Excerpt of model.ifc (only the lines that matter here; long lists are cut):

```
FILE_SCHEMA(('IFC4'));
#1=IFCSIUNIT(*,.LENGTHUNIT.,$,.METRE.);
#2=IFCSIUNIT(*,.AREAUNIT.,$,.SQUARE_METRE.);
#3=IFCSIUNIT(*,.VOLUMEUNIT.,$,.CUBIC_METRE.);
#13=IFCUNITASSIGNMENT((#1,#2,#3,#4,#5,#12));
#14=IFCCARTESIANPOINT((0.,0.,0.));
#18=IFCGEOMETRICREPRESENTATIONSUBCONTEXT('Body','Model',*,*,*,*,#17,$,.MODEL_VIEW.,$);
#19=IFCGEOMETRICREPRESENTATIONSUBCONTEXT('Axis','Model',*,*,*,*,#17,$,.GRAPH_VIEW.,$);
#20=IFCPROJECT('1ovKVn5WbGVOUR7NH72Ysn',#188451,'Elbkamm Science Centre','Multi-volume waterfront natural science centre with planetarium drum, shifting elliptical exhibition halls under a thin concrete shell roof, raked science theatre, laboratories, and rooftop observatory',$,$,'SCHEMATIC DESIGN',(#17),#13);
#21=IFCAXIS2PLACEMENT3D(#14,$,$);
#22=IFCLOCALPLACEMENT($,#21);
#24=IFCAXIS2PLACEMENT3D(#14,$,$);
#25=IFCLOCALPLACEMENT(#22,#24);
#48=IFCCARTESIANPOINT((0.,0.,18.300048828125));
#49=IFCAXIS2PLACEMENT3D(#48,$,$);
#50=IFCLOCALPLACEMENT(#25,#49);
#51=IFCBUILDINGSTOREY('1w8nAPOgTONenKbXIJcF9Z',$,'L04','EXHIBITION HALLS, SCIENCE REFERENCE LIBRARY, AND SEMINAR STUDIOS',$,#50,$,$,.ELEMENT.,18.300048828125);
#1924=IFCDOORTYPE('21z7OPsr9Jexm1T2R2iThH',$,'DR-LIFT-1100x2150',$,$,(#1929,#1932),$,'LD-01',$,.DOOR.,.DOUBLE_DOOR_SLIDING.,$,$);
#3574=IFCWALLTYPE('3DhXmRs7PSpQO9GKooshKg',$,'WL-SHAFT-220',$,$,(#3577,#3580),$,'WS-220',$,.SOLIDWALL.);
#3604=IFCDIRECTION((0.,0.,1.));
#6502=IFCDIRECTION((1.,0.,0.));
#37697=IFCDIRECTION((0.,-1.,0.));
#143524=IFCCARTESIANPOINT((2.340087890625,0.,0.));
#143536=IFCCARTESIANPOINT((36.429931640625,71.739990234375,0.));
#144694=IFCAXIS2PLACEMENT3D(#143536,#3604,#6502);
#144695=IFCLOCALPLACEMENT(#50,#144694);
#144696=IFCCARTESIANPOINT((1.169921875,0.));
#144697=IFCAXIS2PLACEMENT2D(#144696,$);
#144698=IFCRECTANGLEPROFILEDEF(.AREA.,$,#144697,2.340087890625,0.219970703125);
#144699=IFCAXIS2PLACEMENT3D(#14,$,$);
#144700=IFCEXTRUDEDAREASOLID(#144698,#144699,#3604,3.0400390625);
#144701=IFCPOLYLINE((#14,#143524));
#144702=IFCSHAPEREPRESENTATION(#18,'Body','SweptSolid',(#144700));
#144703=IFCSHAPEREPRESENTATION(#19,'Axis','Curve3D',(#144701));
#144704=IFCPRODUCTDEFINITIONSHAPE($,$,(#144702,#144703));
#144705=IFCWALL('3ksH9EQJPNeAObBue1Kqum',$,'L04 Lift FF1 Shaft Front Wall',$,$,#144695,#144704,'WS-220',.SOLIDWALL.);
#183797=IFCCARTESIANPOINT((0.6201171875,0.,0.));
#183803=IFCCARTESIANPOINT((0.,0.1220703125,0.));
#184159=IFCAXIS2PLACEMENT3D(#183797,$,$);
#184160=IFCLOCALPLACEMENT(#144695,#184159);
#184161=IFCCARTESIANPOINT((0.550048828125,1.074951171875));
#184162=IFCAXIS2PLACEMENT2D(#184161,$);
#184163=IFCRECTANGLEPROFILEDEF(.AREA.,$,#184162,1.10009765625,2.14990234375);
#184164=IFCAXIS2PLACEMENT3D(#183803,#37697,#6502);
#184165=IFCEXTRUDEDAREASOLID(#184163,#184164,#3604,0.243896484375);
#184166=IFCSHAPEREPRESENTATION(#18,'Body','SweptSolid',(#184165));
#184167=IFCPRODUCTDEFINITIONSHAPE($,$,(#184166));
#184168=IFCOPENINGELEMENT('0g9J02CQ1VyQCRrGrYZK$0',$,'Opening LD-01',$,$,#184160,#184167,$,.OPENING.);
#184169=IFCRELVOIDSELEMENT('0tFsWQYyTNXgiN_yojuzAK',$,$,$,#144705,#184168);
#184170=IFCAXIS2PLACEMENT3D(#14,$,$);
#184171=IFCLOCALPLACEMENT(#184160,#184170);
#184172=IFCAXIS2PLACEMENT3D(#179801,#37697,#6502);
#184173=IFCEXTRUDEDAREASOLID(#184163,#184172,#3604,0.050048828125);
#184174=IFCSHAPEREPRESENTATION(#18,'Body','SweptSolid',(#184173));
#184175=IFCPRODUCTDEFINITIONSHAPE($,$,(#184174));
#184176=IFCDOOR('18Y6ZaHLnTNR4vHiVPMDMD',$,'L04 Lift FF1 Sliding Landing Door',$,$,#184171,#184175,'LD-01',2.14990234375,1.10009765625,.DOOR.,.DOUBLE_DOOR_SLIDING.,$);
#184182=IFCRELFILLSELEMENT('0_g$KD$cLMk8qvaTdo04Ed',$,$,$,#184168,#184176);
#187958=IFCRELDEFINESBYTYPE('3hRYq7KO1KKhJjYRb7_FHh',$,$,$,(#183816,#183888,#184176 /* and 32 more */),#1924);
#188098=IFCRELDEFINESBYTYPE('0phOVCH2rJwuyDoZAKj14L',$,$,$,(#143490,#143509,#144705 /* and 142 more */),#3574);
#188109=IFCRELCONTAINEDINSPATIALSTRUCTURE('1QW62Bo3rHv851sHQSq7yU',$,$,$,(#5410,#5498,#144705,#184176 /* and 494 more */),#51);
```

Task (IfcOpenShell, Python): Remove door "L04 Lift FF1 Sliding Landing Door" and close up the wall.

```python
import ifcopenshell
import ifcopenshell.api.feature
import ifcopenshell.api.root
import ifcopenshell.geom
import ifcopenshell.util.shape

model = ifcopenshell.open("model.ifc")
settings = ifcopenshell.geom.settings()


def volume(element):
    """Net volume in cubic metres, openings subtracted."""
    shape = ifcopenshell.geom.create_shape(settings, element)
    return ifcopenshell.util.shape.get_volume(shape.geometry)


door = model.by_id(184176)
opening = door.FillsVoids[0].RelatingOpeningElement
wall = opening.VoidsElements[0].RelatingBuildingElement
before = volume(wall)

ifcopenshell.api.root.remove_product(model, product=door)
ifcopenshell.api.feature.remove_feature(model, feature=opening)

after = volume(wall)

print(f"wall volume {before:.3f} -> {after:.3f} m3")

model.write("model_edited.ifc")
```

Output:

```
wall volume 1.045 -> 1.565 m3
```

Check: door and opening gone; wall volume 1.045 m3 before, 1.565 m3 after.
